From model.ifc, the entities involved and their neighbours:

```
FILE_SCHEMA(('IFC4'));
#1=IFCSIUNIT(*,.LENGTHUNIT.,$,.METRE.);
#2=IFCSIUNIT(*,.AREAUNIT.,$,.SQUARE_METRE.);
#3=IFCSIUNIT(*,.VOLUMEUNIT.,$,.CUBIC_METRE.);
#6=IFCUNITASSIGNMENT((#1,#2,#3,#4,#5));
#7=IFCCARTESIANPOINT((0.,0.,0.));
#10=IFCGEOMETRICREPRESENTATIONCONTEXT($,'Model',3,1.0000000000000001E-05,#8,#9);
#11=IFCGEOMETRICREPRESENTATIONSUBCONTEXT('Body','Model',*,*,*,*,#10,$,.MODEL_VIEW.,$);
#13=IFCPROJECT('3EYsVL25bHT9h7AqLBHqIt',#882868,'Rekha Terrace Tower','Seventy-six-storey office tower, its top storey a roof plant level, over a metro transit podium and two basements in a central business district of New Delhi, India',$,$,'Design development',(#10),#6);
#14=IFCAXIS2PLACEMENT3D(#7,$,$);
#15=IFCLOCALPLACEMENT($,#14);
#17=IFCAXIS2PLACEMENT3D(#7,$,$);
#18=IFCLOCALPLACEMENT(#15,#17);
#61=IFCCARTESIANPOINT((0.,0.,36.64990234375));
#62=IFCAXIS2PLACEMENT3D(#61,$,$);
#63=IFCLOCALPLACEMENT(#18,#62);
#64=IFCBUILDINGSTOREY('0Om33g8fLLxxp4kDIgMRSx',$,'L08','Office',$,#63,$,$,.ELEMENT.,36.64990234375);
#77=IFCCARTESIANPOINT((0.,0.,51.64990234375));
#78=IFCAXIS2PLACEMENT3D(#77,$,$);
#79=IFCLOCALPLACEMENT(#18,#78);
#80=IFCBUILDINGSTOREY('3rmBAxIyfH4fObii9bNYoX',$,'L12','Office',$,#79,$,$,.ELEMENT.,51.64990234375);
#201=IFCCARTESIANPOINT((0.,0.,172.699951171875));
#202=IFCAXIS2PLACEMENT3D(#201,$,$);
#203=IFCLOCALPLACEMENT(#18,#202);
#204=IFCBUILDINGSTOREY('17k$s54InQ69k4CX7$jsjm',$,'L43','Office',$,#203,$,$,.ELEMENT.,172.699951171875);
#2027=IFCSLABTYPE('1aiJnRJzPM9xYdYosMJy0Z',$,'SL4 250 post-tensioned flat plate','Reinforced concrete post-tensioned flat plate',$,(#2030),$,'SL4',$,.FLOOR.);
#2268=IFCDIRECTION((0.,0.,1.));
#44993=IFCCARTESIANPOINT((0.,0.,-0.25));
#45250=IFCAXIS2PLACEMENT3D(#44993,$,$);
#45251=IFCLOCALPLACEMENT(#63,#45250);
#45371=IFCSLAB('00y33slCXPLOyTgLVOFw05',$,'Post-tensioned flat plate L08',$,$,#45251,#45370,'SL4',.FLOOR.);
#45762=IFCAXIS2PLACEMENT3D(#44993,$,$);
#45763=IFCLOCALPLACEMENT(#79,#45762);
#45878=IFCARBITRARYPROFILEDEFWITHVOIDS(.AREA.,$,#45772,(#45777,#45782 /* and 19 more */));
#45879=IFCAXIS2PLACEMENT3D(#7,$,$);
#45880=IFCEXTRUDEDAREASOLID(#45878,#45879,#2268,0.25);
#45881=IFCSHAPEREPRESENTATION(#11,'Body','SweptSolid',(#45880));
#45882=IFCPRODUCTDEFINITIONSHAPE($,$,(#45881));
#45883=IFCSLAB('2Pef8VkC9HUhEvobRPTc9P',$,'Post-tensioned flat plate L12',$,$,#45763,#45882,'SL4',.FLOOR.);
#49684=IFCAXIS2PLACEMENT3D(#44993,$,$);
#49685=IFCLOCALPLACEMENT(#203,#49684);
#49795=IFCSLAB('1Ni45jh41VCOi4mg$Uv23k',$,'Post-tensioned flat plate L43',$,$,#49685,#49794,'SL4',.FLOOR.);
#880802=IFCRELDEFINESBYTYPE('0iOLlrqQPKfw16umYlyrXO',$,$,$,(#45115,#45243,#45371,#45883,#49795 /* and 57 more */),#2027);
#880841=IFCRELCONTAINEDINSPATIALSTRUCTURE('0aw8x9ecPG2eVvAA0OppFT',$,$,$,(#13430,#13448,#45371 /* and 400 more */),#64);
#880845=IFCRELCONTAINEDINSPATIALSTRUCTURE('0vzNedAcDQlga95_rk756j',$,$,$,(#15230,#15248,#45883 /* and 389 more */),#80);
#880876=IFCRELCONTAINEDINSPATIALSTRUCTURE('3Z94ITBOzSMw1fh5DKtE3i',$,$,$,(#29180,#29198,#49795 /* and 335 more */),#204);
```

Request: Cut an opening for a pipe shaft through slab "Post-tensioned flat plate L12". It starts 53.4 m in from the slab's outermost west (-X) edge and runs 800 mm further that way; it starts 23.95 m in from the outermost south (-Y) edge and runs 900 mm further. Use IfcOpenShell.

```python
import numpy as np
import ifcopenshell
import ifcopenshell.api.feature
import ifcopenshell.api.geometry
import ifcopenshell.api.root
import ifcopenshell.geom
import ifcopenshell.util.placement
import ifcopenshell.util.representation
import ifcopenshell.util.shape
import ifcopenshell.util.unit

model = ifcopenshell.open("model.ifc")
unit_scale = ifcopenshell.util.unit.calculate_unit_scale(model)
settings = ifcopenshell.geom.settings()


def volume(element):
    """Net volume in cubic metres, openings subtracted."""
    shape = ifcopenshell.geom.create_shape(settings, element)
    return ifcopenshell.util.shape.get_volume(shape.geometry)


slab = model.by_guid("2Pef8VkC9HUhEvobRPTc9P")
before = volume(slab)

# Extent in the slab's own axes, in metres. The edges named are its -X and -Y sides.
slab_shape = ifcopenshell.geom.create_shape(settings, slab)
vertices = ifcopenshell.util.shape.get_vertices(slab_shape.geometry)
x_min, y_min, bottom = vertices.min(axis=0)
top = vertices[:, 2].max()

opening = ifcopenshell.api.root.create_entity(model, ifc_class="IfcOpeningElement", name="Pipe shaft opening", predefined_type="OPENING")
context = ifcopenshell.util.representation.get_context(model, "Model", "Body", "MODEL_VIEW")
width, depth = 0.8, 0.9
outline = [(0.0, 0.0), (width, 0.0), (width, depth), (0.0, depth), (0.0, 0.0)]
# Overshoot both faces by 50 mm so the cut is clean.
shape = ifcopenshell.api.geometry.add_slab_representation(
    model, context=context, depth=top - bottom + 0.1, polyline=outline
)
ifcopenshell.api.geometry.assign_representation(model, product=opening, representation=shape)

matrix = ifcopenshell.util.placement.get_local_placement(slab.ObjectPlacement)
matrix[:, 3] = matrix @ np.append(np.array([x_min + 53.4, y_min + 23.95, bottom - 0.05]) / unit_scale, 1.0)
ifcopenshell.api.geometry.edit_object_placement(model, product=opening, matrix=matrix, is_si=False)
ifcopenshell.api.feature.add_feature(model, feature=opening, element=slab)

after = volume(slab)

print(f"slab volume {before:.3f} -> {after:.3f} m3")

model.write("model_v2.ifc")
```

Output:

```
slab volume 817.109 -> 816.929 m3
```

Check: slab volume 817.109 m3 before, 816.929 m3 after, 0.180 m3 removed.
